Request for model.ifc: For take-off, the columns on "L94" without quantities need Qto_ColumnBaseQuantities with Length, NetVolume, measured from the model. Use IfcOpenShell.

First a look at what the model holds.

```python
import ifcopenshell
import ifcopenshell.util.element
import ifcopenshell.util.unit

model = ifcopenshell.open("model.ifc")
print(model.schema)
for unit_type in ("LENGTHUNIT", "AREAUNIT", "VOLUMEUNIT"):
    print(unit_type, ifcopenshell.util.unit.calculate_unit_scale(model, unit_type))
storey = next(s for s in model.by_type("IfcBuildingStorey") if s.Name == "L94")
columns = [e for e in ifcopenshell.util.element.get_decomposition(storey) if e.is_a("IfcColumn")]
for e in sorted(columns, key=lambda e: e.id()):
    print(e.id(), e.is_a(), e.Name, list(ifcopenshell.util.element.get_psets(e, qtos_only=True)), sep=" | ")
```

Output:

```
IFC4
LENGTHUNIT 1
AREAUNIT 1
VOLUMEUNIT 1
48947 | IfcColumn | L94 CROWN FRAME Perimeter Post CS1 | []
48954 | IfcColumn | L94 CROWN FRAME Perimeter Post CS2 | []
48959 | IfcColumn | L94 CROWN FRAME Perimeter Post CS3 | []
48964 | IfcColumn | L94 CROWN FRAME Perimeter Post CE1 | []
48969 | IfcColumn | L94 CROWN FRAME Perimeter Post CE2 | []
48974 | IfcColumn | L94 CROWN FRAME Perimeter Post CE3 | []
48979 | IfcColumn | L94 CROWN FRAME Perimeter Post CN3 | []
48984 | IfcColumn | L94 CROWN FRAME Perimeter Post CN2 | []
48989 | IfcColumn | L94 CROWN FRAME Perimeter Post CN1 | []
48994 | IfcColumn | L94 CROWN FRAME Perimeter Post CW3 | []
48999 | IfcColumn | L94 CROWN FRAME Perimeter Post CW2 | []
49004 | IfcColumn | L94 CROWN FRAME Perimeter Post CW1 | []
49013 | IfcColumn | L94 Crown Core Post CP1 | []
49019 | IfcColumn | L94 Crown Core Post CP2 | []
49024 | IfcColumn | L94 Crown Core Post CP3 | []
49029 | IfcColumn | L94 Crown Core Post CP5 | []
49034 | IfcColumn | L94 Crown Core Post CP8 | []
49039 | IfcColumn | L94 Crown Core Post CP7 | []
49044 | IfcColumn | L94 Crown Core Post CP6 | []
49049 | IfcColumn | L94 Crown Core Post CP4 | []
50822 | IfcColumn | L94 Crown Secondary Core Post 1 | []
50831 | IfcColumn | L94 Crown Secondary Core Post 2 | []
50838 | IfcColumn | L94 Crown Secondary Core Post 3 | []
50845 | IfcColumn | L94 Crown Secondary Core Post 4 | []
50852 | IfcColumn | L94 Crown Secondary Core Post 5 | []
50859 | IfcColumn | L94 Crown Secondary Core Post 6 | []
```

```python
import ifcopenshell
import ifcopenshell.api.pset
import ifcopenshell.geom
import ifcopenshell.util.element
import ifcopenshell.util.shape
import ifcopenshell.util.unit

model = ifcopenshell.open("model.ifc")
unit_scale = ifcopenshell.util.unit.calculate_unit_scale(model)
volume_scale = ifcopenshell.util.unit.calculate_unit_scale(model, "VOLUMEUNIT")
settings = ifcopenshell.geom.settings()

storey = next(s for s in model.by_type("IfcBuildingStorey") if s.Name == "L94")
columns = [e for e in ifcopenshell.util.element.get_decomposition(storey) if e.is_a("IfcColumn")]

for e in sorted(columns, key=lambda e: e.id()):
    if ifcopenshell.util.element.get_psets(e, qtos_only=True, should_inherit=False):
        continue
    # Geometry comes back in metres, in the element's own axes.
    shape = ifcopenshell.geom.create_shape(settings, e)
    values = {
        "Length": ifcopenshell.util.shape.get_z(shape.geometry) / unit_scale,
        "NetVolume": ifcopenshell.util.shape.get_volume(shape.geometry) / volume_scale,
    }
    qto = ifcopenshell.api.pset.add_qto(model, product=e, name="Qto_ColumnBaseQuantities")
    ifcopenshell.api.pset.edit_qto(model, qto=qto, properties=values)
    print(e.id(), {k: round(v, 3) for k, v in values.items()})

model.write("model_edited.ifc")
```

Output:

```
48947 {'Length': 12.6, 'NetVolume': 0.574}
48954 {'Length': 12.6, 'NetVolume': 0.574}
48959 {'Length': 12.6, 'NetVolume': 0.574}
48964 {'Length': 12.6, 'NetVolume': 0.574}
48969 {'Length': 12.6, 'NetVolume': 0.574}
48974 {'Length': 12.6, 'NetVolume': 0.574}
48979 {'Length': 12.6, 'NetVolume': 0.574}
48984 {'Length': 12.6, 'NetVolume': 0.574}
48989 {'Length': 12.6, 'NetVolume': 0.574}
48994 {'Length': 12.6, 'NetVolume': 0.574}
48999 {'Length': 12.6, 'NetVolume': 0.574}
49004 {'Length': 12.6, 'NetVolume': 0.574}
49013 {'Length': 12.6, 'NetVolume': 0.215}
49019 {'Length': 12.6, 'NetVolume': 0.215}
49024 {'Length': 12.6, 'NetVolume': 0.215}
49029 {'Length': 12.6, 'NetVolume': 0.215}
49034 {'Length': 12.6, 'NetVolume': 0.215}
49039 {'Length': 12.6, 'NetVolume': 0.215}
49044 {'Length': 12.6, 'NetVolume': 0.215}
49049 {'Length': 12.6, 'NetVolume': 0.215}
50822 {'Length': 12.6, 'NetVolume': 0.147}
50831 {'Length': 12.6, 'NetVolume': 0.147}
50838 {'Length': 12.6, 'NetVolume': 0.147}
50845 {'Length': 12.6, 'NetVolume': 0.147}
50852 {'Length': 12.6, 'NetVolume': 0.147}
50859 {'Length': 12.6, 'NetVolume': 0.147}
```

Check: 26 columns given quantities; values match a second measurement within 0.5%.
